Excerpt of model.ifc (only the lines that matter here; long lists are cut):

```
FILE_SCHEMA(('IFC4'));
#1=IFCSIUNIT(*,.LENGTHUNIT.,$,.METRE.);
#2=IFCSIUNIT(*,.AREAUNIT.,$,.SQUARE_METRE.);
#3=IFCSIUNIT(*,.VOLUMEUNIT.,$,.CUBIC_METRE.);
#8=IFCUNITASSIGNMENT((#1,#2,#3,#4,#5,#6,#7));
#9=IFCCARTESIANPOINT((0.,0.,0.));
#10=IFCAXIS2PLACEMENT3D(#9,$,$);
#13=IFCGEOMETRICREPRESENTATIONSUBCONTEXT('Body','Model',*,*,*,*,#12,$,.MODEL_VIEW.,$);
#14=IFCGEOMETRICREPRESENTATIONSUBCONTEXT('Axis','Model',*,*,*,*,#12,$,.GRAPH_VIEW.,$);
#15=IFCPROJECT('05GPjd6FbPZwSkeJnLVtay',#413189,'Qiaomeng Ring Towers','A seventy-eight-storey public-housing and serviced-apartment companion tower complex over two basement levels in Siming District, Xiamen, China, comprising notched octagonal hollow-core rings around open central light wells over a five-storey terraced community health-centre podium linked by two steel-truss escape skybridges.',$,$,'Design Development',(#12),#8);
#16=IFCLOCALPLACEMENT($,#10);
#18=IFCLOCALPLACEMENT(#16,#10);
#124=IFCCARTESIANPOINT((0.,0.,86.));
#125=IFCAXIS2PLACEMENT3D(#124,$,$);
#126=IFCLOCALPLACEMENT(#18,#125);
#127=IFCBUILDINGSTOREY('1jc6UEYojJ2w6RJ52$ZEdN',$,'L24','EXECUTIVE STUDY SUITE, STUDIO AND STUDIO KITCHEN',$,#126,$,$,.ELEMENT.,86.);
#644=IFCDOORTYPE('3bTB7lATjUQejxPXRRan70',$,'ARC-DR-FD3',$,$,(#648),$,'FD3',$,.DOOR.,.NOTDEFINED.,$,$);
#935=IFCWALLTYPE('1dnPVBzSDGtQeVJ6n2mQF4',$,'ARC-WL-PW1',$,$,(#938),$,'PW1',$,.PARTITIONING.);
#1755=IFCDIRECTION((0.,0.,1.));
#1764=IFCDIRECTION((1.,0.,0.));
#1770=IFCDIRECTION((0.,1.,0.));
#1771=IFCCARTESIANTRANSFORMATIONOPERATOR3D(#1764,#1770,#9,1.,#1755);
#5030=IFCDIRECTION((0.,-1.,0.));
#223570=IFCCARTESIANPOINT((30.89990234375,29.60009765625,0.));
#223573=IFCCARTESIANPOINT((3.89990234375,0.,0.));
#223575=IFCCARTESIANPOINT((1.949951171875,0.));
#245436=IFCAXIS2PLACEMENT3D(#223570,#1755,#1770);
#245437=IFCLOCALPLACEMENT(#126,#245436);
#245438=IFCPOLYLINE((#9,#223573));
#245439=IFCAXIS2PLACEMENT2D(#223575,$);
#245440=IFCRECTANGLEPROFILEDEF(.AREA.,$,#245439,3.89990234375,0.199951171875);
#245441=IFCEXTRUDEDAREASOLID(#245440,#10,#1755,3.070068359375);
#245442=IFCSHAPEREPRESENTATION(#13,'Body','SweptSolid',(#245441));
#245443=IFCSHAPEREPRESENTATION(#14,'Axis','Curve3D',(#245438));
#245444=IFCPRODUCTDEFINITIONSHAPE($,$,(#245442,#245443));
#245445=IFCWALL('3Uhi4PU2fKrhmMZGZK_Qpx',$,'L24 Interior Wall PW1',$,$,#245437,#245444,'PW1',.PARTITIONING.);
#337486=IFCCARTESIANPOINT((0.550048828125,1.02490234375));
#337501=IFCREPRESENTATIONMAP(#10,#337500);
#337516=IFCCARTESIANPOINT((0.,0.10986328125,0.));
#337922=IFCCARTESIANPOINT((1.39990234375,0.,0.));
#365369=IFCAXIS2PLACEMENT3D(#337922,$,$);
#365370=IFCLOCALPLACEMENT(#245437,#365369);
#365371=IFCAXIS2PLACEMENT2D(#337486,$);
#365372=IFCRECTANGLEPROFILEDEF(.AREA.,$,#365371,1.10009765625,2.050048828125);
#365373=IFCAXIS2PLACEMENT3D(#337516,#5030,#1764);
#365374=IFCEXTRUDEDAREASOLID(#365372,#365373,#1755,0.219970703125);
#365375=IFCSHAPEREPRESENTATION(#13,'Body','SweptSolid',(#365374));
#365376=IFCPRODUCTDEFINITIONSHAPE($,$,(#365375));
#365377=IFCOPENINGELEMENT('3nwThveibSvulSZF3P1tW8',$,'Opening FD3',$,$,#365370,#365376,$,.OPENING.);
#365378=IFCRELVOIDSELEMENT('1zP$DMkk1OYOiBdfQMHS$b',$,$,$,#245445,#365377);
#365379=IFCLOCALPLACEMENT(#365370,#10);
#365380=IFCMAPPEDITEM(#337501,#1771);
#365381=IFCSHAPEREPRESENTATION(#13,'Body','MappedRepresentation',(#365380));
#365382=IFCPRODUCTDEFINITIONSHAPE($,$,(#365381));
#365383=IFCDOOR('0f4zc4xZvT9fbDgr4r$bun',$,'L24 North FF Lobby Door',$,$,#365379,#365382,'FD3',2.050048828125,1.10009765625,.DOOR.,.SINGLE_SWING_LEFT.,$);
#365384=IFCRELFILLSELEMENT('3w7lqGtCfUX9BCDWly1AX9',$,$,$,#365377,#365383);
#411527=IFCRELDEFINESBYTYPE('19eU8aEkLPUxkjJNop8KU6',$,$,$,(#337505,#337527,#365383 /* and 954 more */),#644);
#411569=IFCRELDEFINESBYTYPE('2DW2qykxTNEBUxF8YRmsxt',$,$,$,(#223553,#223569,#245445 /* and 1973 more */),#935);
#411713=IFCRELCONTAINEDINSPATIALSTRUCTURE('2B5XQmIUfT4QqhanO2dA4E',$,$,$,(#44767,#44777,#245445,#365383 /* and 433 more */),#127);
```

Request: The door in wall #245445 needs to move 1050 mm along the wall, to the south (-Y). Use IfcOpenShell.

```python
import ifcopenshell
import ifcopenshell.api.geometry
import ifcopenshell.util.placement
import ifcopenshell.util.unit

model = ifcopenshell.open("model.ifc")
unit_scale = ifcopenshell.util.unit.calculate_unit_scale(model)

door = model.by_guid("0f4zc4xZvT9fbDgr4r$bun")
opening = door.FillsVoids[0].RelatingOpeningElement
wall = opening.VoidsElements[0].RelatingBuildingElement

wall_matrix = ifcopenshell.util.placement.get_local_placement(wall.ObjectPlacement)
shift = wall_matrix[:3, 0] * -1.05 / unit_scale
before = ifcopenshell.util.placement.get_local_placement(door.ObjectPlacement)[:3, 3].copy()

# The door is placed relative to its opening, so it follows when the opening moves.
matrix = ifcopenshell.util.placement.get_local_placement(opening.ObjectPlacement)
matrix[:3, 3] += shift
ifcopenshell.api.geometry.edit_object_placement(
    model, product=opening, matrix=matrix, is_si=False, should_transform_children=True
)

after = ifcopenshell.util.placement.get_local_placement(door.ObjectPlacement)[:3, 3]
print("door moved by", (after - before).round(3) + 0.0)

model.write("model_edited.ifc")
```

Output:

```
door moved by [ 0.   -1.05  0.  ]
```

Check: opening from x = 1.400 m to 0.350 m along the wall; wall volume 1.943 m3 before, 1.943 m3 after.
